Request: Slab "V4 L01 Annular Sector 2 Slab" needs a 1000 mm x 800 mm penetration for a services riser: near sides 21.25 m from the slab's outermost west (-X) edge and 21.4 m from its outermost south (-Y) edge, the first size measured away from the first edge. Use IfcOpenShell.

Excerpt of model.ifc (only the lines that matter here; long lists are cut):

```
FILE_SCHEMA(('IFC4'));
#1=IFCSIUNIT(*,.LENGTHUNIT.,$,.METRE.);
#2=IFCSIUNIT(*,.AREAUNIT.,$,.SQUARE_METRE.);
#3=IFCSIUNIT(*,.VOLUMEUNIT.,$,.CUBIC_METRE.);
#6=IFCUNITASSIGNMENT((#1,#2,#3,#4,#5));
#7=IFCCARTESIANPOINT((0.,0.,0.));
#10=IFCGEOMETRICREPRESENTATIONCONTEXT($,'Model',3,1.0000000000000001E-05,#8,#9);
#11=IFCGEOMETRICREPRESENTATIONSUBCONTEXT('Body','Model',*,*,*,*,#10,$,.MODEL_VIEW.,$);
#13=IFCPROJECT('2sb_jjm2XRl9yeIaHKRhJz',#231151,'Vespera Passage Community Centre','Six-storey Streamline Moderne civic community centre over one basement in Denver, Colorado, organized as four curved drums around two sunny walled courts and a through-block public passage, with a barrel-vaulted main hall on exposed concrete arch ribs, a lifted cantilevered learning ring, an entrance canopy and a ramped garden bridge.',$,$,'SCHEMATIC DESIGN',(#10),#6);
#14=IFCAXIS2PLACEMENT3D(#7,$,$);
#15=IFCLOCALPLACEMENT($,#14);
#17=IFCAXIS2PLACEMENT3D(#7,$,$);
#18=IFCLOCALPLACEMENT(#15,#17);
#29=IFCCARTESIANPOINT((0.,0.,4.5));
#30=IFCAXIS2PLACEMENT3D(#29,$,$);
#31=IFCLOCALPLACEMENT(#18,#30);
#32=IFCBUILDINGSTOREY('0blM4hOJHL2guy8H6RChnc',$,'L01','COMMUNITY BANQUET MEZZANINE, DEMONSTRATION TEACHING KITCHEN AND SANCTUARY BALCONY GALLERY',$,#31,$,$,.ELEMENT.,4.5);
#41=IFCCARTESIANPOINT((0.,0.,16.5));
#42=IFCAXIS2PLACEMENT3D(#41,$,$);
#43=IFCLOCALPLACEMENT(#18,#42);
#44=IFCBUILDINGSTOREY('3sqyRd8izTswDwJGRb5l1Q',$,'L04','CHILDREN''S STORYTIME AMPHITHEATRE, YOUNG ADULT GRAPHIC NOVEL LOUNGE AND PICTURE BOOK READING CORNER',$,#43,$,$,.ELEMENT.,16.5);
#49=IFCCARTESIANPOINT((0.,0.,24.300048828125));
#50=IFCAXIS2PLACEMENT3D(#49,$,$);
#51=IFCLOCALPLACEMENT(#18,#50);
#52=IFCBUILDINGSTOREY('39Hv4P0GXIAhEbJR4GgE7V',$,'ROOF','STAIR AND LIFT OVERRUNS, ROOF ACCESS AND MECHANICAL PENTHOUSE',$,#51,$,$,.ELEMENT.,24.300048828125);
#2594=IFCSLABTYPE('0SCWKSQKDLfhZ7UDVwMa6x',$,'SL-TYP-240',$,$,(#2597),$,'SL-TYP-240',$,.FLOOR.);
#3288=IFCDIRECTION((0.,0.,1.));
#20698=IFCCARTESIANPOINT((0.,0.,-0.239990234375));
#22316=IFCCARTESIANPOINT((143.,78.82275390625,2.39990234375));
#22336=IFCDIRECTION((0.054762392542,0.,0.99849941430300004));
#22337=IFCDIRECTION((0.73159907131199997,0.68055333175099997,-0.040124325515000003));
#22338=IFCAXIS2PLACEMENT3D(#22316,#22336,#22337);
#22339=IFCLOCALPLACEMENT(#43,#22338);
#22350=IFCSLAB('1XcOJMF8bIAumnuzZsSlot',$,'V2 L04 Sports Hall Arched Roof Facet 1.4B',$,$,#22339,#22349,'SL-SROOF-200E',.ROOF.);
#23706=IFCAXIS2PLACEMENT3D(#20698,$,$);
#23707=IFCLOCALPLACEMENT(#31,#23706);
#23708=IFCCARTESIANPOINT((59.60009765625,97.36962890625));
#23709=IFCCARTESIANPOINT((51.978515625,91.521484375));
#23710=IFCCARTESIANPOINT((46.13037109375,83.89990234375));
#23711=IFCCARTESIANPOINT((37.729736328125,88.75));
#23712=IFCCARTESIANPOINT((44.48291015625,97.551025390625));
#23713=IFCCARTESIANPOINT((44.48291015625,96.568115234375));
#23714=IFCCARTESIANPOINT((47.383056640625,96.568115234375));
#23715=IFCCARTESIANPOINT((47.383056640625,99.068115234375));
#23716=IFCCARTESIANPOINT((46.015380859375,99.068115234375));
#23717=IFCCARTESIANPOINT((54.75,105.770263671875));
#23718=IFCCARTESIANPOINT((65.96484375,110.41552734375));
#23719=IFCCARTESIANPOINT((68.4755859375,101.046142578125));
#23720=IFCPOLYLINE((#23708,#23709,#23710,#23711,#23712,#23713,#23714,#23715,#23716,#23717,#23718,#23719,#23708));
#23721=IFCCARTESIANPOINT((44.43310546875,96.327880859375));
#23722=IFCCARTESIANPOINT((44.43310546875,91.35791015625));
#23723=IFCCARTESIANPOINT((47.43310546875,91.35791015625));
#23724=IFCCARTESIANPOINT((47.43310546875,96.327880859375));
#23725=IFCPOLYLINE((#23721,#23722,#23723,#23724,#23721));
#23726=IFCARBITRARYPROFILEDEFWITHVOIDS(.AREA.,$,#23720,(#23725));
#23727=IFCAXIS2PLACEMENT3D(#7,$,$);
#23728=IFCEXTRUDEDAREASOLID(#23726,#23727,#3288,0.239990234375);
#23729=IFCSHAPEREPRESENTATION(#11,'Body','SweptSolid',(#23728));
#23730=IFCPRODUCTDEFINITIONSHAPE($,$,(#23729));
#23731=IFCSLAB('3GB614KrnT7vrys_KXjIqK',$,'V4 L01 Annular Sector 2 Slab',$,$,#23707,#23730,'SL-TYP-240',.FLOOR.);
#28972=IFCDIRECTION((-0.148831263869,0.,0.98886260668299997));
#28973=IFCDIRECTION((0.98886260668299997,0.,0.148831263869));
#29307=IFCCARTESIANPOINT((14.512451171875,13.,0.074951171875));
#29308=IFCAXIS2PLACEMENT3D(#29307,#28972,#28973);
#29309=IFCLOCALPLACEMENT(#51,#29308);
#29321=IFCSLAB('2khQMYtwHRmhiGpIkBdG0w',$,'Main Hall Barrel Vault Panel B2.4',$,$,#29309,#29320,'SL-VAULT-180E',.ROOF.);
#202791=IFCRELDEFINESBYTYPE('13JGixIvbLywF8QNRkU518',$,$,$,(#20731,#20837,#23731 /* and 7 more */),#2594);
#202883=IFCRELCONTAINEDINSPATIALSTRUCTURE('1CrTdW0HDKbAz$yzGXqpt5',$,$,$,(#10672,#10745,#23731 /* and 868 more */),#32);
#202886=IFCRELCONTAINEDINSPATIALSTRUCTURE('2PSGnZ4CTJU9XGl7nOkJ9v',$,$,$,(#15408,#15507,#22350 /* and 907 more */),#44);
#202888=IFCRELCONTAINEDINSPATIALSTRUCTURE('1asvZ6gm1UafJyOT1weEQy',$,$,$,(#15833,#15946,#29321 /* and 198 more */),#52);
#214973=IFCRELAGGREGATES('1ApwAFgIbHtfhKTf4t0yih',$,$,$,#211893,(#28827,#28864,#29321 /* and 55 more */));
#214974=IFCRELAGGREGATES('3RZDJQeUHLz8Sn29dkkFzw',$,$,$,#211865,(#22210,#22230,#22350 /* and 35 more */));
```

```python
import numpy as np
import ifcopenshell
import ifcopenshell.api.feature
import ifcopenshell.api.geometry
import ifcopenshell.api.root
import ifcopenshell.geom
import ifcopenshell.util.placement
import ifcopenshell.util.representation
import ifcopenshell.util.shape
import ifcopenshell.util.unit

model = ifcopenshell.open("model.ifc")
unit_scale = ifcopenshell.util.unit.calculate_unit_scale(model)
settings = ifcopenshell.geom.settings()


def volume(element):
    """Net volume in cubic metres, openings subtracted."""
    shape = ifcopenshell.geom.create_shape(settings, element)
    return ifcopenshell.util.shape.get_volume(shape.geometry)


slab = model.by_guid("3GB614KrnT7vrys_KXjIqK")
before = volume(slab)

# Extent in the slab's own axes, in metres. The edges named are its -X and -Y sides.
slab_shape = ifcopenshell.geom.create_shape(settings, slab)
vertices = ifcopenshell.util.shape.get_vertices(slab_shape.geometry)
x_min, y_min, bottom = vertices.min(axis=0)
top = vertices[:, 2].max()

opening = ifcopenshell.api.root.create_entity(model, ifc_class="IfcOpeningElement", name="Services riser opening", predefined_type="OPENING")
context = ifcopenshell.util.representation.get_context(model, "Model", "Body", "MODEL_VIEW")
width, depth = 1, 0.8
outline = [(0.0, 0.0), (width, 0.0), (width, depth), (0.0, depth), (0.0, 0.0)]
# Overshoot both faces by 50 mm so the cut is clean.
shape = ifcopenshell.api.geometry.add_slab_representation(
    model, context=context, depth=top - bottom + 0.1, polyline=outline
)
ifcopenshell.api.geometry.assign_representation(model, product=opening, representation=shape)

matrix = ifcopenshell.util.placement.get_local_placement(slab.ObjectPlacement)
matrix[:, 3] = matrix @ np.append(np.array([x_min + 21.25, y_min + 21.4, bottom - 0.05]) / unit_scale, 1.0)
ifcopenshell.api.geometry.edit_object_placement(model, product=opening, matrix=matrix, is_si=False)
ifcopenshell.api.feature.add_feature(model, feature=opening, element=slab)

after = volume(slab)

print(f"slab volume {before:.3f} -> {after:.3f} m3")

model.write("model_rev.ifc")
```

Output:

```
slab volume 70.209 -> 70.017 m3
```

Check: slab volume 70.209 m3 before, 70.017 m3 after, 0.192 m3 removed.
